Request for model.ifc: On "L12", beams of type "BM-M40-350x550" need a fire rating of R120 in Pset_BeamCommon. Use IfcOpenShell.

First a look at what the model holds.

```python
import ifcopenshell
import ifcopenshell.util.element

model = ifcopenshell.open("model.ifc")
print(model.schema)
storey = next(s for s in model.by_type("IfcBuildingStorey") if s.Name == "L12")
beams = [e for e in ifcopenshell.util.element.get_decomposition(storey) if e.is_a("IfcBeam")]
seen = {}
for e in beams:
    element_type = ifcopenshell.util.element.get_type(e)
    key = (element_type.Name if element_type != e and element_type else None, ifcopenshell.util.element.get_pset(e, "Pset_BeamCommon", "FireRating"))
    seen[key] = seen.get(key, 0) + 1
for (name, value), count in sorted(seen.items(), key=str):
    print(count, "x", name, "|", value)
```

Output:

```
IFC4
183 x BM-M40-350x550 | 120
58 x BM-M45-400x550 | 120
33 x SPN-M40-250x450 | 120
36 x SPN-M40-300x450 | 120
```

```python
import ifcopenshell
import ifcopenshell.api.pset
import ifcopenshell.util.element

model = ifcopenshell.open("model.ifc")

storey = next(s for s in model.by_type("IfcBuildingStorey") if s.Name == "L12")
beams = [e for e in ifcopenshell.util.element.get_decomposition(storey) if e.is_a("IfcBeam")]

count = 0
for e in beams:
    element_type = ifcopenshell.util.element.get_type(e)
    if element_type in (None, e) or element_type.Name != "BM-M40-350x550":
        continue
    # add_pset returns the element's existing set when there is one.
    pset = ifcopenshell.api.pset.add_pset(model, product=e, name="Pset_BeamCommon")
    ifcopenshell.api.pset.edit_pset(model, pset=pset, properties={"FireRating": "R120"})
    count += 1

print(count, "beams updated")

model.write("model_v2.ifc")
```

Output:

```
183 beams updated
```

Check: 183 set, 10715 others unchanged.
